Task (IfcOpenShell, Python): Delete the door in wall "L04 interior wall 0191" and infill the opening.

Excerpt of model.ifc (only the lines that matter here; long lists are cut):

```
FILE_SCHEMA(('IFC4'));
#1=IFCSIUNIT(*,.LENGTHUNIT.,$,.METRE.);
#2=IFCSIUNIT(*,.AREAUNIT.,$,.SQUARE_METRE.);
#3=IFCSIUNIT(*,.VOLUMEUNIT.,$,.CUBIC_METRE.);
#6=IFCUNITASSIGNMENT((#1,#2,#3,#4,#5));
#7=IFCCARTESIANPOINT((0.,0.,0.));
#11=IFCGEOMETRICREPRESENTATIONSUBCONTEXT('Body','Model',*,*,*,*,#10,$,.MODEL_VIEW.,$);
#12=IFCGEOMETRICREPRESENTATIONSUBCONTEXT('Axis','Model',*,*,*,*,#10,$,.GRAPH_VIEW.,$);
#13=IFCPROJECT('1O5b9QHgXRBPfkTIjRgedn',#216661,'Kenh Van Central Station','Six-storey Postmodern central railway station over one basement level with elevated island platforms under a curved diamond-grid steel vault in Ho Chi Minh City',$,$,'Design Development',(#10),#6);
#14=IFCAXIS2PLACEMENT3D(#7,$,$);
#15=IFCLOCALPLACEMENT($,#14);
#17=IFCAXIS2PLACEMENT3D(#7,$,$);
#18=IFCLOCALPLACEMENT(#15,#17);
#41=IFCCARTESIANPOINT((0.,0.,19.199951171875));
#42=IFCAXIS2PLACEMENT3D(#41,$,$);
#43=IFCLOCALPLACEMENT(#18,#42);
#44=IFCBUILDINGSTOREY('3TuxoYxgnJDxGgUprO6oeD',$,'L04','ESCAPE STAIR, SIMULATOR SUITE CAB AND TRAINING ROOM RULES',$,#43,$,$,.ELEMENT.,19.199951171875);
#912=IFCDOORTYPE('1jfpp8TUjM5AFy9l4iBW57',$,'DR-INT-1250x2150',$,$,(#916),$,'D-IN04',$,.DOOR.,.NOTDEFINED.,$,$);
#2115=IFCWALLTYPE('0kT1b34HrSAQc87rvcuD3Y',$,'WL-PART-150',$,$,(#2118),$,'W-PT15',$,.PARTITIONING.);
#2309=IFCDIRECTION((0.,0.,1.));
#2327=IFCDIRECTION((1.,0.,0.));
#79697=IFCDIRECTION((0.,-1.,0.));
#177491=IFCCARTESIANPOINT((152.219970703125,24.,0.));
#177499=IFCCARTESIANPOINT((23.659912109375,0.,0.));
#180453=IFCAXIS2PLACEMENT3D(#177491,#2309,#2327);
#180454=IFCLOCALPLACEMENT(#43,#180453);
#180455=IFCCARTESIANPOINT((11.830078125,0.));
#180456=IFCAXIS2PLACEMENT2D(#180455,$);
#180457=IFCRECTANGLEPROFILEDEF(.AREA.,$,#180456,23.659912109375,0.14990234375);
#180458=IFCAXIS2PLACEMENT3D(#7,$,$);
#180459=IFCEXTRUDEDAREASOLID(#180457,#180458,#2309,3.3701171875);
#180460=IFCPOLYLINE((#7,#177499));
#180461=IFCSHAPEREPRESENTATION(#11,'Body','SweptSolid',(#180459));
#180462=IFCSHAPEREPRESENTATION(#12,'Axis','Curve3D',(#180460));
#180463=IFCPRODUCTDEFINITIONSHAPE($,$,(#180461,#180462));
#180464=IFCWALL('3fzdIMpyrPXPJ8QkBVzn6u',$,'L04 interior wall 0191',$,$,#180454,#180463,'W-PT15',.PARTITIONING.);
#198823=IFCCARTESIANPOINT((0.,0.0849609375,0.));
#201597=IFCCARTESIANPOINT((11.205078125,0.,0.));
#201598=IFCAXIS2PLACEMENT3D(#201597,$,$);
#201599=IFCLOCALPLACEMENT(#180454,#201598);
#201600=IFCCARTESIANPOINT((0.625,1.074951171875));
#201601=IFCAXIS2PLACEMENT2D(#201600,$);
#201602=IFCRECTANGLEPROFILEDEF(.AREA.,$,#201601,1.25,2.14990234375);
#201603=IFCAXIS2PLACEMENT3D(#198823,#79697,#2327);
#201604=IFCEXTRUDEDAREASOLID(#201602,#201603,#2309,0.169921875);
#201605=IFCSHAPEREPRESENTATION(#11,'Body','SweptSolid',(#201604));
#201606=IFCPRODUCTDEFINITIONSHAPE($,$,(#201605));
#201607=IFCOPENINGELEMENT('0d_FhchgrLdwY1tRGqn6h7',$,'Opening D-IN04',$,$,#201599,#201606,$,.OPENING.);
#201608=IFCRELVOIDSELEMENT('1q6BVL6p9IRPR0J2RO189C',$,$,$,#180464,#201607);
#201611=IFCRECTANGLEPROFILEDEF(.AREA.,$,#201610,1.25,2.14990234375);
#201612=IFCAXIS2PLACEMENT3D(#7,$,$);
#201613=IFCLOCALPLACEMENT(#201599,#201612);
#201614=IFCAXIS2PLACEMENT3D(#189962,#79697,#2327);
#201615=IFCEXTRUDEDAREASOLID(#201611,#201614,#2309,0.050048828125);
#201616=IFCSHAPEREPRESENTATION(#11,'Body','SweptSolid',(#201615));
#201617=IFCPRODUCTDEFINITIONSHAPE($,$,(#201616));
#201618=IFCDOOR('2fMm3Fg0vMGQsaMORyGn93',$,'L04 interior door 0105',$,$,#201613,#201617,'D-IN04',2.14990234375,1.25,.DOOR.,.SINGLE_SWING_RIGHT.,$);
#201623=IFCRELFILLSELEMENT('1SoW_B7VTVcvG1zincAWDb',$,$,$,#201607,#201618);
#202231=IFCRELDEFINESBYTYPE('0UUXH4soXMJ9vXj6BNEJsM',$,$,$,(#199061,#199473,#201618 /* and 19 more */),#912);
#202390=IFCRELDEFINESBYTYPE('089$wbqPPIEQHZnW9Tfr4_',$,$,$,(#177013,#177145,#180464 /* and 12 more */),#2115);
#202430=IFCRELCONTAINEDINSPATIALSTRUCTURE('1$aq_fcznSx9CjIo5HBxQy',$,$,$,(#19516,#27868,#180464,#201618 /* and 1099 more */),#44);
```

```python
import ifcopenshell
import ifcopenshell.api.feature
import ifcopenshell.api.root
import ifcopenshell.geom
import ifcopenshell.util.shape

model = ifcopenshell.open("model.ifc")
settings = ifcopenshell.geom.settings()


def volume(element):
    """Net volume in cubic metres, openings subtracted."""
    shape = ifcopenshell.geom.create_shape(settings, element)
    return ifcopenshell.util.shape.get_volume(shape.geometry)


door = model.by_guid("2fMm3Fg0vMGQsaMORyGn93")
opening = door.FillsVoids[0].RelatingOpeningElement
wall = opening.VoidsElements[0].RelatingBuildingElement
before = volume(wall)

ifcopenshell.api.root.remove_product(model, product=door)
ifcopenshell.api.feature.remove_feature(model, feature=opening)

after = volume(wall)

print(f"wall volume {before:.3f} -> {after:.3f} m3")

model.write("model-out.ifc")
```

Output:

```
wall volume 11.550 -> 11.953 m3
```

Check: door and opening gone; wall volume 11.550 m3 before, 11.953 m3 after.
